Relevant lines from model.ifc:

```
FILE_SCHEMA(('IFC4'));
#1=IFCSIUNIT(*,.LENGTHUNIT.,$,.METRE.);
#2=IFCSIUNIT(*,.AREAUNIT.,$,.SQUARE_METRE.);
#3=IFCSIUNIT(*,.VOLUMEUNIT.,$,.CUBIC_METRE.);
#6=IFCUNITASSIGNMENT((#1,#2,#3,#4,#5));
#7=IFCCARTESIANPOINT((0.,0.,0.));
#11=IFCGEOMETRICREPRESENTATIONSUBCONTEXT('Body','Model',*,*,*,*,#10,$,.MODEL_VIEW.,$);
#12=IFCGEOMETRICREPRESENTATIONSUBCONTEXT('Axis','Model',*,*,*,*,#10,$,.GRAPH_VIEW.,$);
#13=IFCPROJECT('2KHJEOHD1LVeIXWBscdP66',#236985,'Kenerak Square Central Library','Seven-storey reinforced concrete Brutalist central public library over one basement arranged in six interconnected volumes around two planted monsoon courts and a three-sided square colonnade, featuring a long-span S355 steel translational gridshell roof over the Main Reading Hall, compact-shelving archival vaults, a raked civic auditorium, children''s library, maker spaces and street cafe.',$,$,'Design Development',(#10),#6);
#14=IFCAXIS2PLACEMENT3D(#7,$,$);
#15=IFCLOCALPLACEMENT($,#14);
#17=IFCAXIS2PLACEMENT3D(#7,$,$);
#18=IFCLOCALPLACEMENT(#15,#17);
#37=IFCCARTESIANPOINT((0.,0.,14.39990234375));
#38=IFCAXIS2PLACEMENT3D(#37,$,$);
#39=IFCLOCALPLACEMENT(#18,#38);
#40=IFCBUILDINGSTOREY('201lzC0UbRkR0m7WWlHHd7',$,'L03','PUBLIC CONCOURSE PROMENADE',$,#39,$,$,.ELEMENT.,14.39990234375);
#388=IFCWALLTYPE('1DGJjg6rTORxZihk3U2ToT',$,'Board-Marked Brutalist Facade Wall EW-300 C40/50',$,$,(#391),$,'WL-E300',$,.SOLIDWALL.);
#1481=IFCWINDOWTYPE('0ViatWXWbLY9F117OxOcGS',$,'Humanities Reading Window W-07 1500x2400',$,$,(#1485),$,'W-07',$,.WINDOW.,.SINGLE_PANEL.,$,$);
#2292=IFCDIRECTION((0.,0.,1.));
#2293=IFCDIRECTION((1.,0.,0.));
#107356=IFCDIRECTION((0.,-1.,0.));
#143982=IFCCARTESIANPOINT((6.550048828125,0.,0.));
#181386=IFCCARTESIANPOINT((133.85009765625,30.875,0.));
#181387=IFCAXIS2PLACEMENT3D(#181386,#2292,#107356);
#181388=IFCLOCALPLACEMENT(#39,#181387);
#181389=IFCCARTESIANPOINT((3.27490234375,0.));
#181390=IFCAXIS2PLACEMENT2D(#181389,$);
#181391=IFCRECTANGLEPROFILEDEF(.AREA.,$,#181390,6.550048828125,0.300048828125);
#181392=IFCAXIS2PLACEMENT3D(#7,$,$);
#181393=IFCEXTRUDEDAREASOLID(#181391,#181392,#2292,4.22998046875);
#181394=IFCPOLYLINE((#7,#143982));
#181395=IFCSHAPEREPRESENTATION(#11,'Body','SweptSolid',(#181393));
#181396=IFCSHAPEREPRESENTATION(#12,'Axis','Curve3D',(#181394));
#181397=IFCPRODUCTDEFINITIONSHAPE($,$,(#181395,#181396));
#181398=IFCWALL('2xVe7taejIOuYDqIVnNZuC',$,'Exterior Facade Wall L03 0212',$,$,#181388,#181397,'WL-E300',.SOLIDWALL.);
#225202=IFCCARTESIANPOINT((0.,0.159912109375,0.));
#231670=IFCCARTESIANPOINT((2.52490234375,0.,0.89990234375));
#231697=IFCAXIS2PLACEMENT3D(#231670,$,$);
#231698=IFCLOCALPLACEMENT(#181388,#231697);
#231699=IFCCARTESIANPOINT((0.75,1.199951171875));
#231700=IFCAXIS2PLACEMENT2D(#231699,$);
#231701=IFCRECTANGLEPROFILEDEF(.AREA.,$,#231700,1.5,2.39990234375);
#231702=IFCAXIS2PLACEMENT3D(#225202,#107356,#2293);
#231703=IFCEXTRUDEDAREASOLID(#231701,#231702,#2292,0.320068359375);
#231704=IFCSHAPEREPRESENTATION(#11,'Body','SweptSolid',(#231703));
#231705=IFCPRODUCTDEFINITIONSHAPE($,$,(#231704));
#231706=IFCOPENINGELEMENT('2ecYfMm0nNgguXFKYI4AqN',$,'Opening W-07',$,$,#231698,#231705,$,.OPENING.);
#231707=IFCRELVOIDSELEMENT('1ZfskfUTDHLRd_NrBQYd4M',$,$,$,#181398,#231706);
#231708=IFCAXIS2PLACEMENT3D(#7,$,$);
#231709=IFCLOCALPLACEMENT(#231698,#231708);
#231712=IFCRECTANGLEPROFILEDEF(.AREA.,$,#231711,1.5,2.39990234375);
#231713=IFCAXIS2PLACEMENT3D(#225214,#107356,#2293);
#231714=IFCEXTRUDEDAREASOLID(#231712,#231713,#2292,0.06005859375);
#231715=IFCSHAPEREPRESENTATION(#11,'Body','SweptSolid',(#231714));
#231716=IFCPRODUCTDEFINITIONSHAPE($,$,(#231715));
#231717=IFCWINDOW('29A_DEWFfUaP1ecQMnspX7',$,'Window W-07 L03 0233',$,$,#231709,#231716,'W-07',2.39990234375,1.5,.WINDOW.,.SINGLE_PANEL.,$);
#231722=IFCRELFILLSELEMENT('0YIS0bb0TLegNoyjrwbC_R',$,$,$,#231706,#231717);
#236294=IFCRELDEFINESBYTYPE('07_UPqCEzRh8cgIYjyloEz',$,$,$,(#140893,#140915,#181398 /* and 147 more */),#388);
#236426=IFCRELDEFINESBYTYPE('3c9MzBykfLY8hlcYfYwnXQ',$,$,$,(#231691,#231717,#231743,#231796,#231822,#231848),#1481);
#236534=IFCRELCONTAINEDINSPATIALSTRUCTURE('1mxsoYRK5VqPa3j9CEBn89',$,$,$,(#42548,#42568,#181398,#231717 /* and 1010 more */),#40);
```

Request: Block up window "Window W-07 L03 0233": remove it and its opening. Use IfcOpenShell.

```python
import ifcopenshell
import ifcopenshell.api.feature
import ifcopenshell.api.root
import ifcopenshell.geom
import ifcopenshell.util.shape

model = ifcopenshell.open("model.ifc")
settings = ifcopenshell.geom.settings()


def volume(element):
    """Net volume in cubic metres, openings subtracted."""
    shape = ifcopenshell.geom.create_shape(settings, element)
    return ifcopenshell.util.shape.get_volume(shape.geometry)


window = model.by_guid("29A_DEWFfUaP1ecQMnspX7")
opening = window.FillsVoids[0].RelatingOpeningElement
wall = opening.VoidsElements[0].RelatingBuildingElement
before = volume(wall)

ifcopenshell.api.root.remove_product(model, product=window)
ifcopenshell.api.feature.remove_feature(model, feature=opening)

after = volume(wall)

print(f"wall volume {before:.3f} -> {after:.3f} m3")

model.write("model-out.ifc")
```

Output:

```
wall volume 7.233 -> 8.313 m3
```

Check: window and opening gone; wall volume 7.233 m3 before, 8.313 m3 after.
